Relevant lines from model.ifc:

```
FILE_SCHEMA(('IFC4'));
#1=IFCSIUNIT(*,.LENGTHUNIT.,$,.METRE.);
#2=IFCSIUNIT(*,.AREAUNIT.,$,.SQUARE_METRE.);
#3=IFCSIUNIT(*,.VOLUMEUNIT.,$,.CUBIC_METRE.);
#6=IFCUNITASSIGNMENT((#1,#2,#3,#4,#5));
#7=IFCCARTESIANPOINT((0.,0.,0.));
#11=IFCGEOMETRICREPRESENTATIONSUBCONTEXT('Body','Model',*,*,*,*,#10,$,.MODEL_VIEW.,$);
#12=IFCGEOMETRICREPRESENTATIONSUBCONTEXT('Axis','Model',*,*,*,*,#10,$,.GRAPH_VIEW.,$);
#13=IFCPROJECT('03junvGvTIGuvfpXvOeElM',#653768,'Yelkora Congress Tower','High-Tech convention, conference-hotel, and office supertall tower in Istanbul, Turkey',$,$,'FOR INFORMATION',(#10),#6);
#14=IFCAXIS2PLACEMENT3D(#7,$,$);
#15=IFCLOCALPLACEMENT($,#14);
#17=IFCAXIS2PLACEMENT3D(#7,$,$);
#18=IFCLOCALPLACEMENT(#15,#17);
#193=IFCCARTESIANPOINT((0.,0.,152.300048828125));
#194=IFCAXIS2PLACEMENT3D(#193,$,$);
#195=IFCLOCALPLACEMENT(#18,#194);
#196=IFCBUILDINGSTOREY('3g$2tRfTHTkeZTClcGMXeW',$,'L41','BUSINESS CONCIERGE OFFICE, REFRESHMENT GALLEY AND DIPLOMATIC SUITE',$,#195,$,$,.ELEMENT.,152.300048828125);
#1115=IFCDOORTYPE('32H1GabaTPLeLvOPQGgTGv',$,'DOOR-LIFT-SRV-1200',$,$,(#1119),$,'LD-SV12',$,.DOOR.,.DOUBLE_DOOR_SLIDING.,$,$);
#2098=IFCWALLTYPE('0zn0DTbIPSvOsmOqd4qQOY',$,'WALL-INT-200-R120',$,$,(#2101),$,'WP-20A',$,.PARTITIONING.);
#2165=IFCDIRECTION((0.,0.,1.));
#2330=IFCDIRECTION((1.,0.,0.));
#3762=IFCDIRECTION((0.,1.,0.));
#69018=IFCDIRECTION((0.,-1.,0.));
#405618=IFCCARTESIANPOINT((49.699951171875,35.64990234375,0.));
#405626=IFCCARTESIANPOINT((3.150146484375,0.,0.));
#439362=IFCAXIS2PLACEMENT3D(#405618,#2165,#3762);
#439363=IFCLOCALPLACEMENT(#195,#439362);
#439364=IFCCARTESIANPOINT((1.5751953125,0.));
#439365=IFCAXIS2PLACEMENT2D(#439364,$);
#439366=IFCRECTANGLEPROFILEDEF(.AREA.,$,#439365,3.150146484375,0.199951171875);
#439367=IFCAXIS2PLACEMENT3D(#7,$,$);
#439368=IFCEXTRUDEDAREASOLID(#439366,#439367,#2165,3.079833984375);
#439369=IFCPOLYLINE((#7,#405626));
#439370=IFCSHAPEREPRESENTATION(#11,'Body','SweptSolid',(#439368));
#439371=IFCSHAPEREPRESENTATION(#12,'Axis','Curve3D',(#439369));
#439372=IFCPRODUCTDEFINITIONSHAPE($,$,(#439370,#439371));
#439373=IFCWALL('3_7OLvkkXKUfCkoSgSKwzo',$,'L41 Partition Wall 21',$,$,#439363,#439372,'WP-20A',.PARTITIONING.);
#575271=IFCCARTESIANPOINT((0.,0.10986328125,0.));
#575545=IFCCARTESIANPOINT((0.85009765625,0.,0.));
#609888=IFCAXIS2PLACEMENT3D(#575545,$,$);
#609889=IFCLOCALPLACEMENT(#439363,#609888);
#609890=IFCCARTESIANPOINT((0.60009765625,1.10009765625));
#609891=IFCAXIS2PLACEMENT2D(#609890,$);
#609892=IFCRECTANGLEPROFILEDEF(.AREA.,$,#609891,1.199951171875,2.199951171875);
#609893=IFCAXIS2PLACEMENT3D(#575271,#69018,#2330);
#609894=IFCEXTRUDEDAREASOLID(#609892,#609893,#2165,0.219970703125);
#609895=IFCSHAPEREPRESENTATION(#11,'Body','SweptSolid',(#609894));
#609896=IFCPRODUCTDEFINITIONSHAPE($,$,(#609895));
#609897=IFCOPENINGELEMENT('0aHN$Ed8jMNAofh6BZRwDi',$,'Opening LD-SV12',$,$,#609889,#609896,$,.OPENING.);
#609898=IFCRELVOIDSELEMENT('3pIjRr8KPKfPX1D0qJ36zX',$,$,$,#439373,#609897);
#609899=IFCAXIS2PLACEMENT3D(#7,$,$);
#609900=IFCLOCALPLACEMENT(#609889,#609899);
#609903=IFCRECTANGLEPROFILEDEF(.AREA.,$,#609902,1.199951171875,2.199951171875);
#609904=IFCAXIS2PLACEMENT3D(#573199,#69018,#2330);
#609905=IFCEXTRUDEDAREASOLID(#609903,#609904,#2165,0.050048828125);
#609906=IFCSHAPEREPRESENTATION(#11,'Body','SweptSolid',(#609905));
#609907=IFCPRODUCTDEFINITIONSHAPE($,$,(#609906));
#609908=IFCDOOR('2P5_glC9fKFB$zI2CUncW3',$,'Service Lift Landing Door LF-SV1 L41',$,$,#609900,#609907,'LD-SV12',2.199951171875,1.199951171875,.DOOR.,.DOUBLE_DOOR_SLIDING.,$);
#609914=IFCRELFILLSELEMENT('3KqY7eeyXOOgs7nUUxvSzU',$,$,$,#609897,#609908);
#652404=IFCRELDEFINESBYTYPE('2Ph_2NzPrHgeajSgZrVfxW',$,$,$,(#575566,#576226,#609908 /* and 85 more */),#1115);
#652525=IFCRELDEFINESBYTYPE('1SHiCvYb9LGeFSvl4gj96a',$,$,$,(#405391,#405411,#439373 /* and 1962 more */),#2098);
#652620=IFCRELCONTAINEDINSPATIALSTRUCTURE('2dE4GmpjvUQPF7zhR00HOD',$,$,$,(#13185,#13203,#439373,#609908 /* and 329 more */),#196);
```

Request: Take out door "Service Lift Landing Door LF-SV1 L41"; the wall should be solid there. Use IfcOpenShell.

```python
import ifcopenshell
import ifcopenshell.api.feature
import ifcopenshell.api.root
import ifcopenshell.geom
import ifcopenshell.util.shape

model = ifcopenshell.open("model.ifc")
settings = ifcopenshell.geom.settings()


def volume(element):
    """Net volume in cubic metres, openings subtracted."""
    shape = ifcopenshell.geom.create_shape(settings, element)
    return ifcopenshell.util.shape.get_volume(shape.geometry)


door = model.by_guid("2P5_glC9fKFB$zI2CUncW3")
opening = door.FillsVoids[0].RelatingOpeningElement
wall = opening.VoidsElements[0].RelatingBuildingElement
before = volume(wall)

ifcopenshell.api.root.remove_product(model, product=door)
ifcopenshell.api.feature.remove_feature(model, feature=opening)

after = volume(wall)

print(f"wall volume {before:.3f} -> {after:.3f} m3")

model.write("model_edited.ifc")
```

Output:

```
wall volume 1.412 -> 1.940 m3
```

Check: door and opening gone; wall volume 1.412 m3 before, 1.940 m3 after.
